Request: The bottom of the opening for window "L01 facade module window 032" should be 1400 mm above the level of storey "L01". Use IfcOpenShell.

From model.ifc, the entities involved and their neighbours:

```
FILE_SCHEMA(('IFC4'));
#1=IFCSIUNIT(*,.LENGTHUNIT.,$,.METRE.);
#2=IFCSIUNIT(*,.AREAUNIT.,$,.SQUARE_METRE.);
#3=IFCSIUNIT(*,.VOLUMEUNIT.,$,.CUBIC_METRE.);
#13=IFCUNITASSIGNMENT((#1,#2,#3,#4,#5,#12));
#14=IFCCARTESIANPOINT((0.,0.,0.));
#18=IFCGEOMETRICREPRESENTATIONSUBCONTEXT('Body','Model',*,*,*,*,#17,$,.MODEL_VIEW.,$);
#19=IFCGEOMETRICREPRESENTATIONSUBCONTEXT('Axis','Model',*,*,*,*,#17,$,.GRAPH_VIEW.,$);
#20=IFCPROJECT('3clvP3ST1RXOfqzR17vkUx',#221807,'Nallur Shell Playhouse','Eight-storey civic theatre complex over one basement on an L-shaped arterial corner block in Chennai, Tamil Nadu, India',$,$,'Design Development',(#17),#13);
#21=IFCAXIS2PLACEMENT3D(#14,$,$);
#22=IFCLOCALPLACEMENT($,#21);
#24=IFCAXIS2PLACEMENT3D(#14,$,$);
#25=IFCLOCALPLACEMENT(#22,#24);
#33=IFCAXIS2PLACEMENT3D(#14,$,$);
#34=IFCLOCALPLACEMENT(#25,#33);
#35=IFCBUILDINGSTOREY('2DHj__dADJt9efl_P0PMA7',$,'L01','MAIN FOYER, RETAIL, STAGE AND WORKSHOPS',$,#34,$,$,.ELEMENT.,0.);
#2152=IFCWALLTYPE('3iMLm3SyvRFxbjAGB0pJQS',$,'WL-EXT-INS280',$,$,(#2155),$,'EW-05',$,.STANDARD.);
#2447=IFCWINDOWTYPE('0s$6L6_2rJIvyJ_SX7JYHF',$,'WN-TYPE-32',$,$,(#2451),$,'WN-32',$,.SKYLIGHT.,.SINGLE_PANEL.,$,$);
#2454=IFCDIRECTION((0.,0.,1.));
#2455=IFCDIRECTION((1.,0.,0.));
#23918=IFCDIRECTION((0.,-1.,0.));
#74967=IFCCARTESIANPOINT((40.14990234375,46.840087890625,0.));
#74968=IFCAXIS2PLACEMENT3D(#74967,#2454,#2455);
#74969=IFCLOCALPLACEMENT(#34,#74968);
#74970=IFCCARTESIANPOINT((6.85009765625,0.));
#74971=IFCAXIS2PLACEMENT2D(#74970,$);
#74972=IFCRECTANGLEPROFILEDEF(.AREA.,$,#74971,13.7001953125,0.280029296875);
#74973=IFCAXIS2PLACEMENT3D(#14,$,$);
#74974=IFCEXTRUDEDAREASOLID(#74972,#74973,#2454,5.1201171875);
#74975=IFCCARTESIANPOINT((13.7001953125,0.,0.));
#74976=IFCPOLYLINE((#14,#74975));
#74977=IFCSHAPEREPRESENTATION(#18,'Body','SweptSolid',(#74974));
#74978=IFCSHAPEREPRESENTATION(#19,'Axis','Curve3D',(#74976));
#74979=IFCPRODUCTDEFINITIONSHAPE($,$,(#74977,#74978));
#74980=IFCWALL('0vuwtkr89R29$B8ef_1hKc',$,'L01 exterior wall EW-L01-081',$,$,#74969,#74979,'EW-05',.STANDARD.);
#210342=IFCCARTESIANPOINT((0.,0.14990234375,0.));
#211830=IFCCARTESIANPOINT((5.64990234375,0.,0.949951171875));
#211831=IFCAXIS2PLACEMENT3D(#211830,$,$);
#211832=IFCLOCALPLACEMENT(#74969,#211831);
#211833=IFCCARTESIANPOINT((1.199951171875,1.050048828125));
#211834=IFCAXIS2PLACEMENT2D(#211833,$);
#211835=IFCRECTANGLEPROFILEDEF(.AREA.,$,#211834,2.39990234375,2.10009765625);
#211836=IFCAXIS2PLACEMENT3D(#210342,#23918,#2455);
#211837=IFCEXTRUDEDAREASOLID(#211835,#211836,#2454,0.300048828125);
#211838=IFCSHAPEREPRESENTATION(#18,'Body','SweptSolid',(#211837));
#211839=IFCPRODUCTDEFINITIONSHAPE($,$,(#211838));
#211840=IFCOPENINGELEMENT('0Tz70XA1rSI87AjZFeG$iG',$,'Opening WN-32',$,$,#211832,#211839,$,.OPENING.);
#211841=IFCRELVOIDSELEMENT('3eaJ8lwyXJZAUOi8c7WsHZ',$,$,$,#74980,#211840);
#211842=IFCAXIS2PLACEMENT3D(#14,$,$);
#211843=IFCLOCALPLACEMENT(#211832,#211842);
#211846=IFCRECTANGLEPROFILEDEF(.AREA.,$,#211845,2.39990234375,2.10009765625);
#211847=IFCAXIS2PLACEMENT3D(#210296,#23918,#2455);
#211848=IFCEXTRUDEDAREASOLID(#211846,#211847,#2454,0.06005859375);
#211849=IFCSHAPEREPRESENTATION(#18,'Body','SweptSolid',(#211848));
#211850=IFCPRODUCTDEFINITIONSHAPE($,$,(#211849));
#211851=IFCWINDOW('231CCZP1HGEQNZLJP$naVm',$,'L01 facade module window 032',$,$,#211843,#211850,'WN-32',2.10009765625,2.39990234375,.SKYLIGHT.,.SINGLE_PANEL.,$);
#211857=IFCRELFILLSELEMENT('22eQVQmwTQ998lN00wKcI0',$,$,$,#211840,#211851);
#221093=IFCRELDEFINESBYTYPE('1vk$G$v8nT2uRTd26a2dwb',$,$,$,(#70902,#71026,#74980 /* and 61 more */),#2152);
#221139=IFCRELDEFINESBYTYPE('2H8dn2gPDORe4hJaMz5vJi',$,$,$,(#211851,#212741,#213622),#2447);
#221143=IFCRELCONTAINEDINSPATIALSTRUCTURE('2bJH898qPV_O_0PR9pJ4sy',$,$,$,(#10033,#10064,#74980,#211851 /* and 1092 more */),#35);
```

```python
import numpy as np
import ifcopenshell
import ifcopenshell.api.geometry
import ifcopenshell.geom
import ifcopenshell.util.element
import ifcopenshell.util.placement
import ifcopenshell.util.shape
import ifcopenshell.util.unit

model = ifcopenshell.open("model.ifc")
unit_scale = ifcopenshell.util.unit.calculate_unit_scale(model)

window = model.by_id(211851)
opening = window.FillsVoids[0].RelatingOpeningElement
storey = ifcopenshell.util.element.get_container(window, ifc_class="IfcBuildingStorey")
level = ifcopenshell.util.placement.get_local_placement(storey.ObjectPlacement)[2, 3]

# The opening's origin need not be at the sill, so measure its lowest point.
shape = ifcopenshell.geom.create_shape(ifcopenshell.geom.settings(), opening)
bottom = ifcopenshell.util.shape.get_shape_bottom_elevation(shape, shape.geometry) / unit_scale
dz = level + 1.4 / unit_scale - bottom

shift = np.array([0.0, 0.0, dz])
# The window is placed relative to its opening, so it follows when the opening moves.
matrix = ifcopenshell.util.placement.get_local_placement(opening.ObjectPlacement)
matrix[:3, 3] += shift
ifcopenshell.api.geometry.edit_object_placement(
    model, product=opening, matrix=matrix, is_si=False, should_transform_children=True
)

print(f"moved by {dz * unit_scale:+.3f} m")

model.write("model_v2.ifc")
```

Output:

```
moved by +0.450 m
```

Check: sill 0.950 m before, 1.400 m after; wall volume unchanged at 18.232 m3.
